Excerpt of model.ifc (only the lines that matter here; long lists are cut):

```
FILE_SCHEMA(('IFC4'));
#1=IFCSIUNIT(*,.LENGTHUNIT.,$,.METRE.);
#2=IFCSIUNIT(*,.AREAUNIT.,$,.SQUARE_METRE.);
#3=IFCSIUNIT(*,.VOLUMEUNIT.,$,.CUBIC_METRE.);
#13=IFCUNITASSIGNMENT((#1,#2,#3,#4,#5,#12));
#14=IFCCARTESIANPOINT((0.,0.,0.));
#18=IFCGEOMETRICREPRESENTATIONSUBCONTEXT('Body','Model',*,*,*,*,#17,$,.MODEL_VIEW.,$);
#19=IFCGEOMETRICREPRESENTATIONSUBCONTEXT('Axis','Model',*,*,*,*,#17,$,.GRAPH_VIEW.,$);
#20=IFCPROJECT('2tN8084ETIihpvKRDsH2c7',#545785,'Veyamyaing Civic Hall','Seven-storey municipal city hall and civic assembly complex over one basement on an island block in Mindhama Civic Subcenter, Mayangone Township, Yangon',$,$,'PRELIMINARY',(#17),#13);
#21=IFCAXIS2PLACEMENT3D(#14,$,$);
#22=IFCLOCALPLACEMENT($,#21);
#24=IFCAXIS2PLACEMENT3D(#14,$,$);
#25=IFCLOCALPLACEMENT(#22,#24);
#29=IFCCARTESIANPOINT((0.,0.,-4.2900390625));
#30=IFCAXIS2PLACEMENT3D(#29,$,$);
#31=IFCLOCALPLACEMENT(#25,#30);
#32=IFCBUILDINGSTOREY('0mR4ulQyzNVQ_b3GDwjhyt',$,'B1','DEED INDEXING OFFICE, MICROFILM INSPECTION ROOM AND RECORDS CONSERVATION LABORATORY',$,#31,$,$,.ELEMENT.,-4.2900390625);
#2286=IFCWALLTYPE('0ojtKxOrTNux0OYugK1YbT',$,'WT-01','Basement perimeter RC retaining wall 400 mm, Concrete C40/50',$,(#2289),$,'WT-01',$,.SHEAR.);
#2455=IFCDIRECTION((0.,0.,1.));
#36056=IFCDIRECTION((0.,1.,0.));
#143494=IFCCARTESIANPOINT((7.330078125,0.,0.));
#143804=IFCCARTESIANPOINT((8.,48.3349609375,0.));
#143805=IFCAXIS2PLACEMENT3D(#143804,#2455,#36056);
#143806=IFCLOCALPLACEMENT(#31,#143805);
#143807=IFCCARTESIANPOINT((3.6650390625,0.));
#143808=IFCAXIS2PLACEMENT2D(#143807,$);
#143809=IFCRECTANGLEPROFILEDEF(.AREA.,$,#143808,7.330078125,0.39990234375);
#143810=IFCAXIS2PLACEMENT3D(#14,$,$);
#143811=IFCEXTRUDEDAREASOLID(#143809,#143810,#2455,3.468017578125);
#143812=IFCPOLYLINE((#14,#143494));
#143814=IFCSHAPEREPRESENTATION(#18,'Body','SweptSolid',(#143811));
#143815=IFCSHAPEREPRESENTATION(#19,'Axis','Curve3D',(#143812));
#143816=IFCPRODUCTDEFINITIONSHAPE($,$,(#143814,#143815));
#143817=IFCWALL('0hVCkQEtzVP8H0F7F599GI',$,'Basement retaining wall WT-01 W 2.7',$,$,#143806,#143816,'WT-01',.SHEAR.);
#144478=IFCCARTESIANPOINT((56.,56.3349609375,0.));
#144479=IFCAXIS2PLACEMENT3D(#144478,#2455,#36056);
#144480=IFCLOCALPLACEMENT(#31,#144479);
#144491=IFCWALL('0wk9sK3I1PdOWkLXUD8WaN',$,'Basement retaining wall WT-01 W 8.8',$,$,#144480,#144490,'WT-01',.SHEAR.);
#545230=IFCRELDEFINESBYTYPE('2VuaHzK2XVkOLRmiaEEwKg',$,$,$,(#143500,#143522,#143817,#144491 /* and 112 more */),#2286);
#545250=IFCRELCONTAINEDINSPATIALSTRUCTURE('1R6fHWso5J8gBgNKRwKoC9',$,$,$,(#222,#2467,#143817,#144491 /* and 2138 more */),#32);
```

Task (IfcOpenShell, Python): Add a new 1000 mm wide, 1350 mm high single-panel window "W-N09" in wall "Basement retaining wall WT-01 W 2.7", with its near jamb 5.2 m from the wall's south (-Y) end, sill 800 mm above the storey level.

```python
import numpy as np
import ifcopenshell
import ifcopenshell.api.feature
import ifcopenshell.api.geometry
import ifcopenshell.api.root
import ifcopenshell.api.spatial
import ifcopenshell.geom
import ifcopenshell.util.element
import ifcopenshell.util.placement
import ifcopenshell.util.representation
import ifcopenshell.util.shape
import ifcopenshell.util.unit

model = ifcopenshell.open("model.ifc")
unit_scale = ifcopenshell.util.unit.calculate_unit_scale(model)
settings = ifcopenshell.geom.settings()


def volume(element):
    """Net volume in cubic metres, openings subtracted."""
    shape = ifcopenshell.geom.create_shape(settings, element)
    return ifcopenshell.util.shape.get_volume(shape.geometry)


wall = model.by_id(143817)
storey = ifcopenshell.util.element.get_container(wall, ifc_class="IfcBuildingStorey")
context = ifcopenshell.util.representation.get_context(model, "Model", "Body", "MODEL_VIEW")
before = volume(wall)

width, height, from_end, sill = 1, 1.35, 5.2, 0.8  # metres

# The wall runs along its own X axis, and the end named is its -X end.
wall_shape = ifcopenshell.geom.create_shape(settings, wall)
x, y, z = ifcopenshell.util.shape.get_vertices(wall_shape.geometry).T
start = x.min() + from_end
face, thickness = float(y.min()), float(y.max() - y.min())
wall_matrix = ifcopenshell.util.placement.get_local_placement(wall.ObjectPlacement)
level = ifcopenshell.util.placement.get_local_placement(storey.ObjectPlacement)[2, 3]


def in_wall(x, y):
    """Placement at x, y metres in the wall's axes, at sill height."""
    matrix = wall_matrix.copy()
    matrix[:, 3] = wall_matrix @ np.array([x / unit_scale, y / unit_scale, 0.0, 1.0])
    matrix[2, 3] = level + sill / unit_scale
    return matrix


# Opening: a box that overshoots both wall faces by 50 mm.
opening = ifcopenshell.api.root.create_entity(model, ifc_class="IfcOpeningElement", predefined_type="OPENING")
box = ifcopenshell.api.geometry.add_wall_representation(
    model, context=context, length=width, height=height, thickness=thickness + 0.1
)
ifcopenshell.api.geometry.assign_representation(model, product=opening, representation=box)
ifcopenshell.api.geometry.edit_object_placement(model, product=opening, matrix=in_wall(start, face - 0.05), is_si=False)
ifcopenshell.api.feature.add_feature(model, feature=opening, element=wall)

window = ifcopenshell.api.root.create_entity(model, ifc_class="IfcWindow", name="W-N09", predefined_type="WINDOW")
window.OverallWidth, window.OverallHeight = width / unit_scale, height / unit_scale
window.PartitioningType = "SINGLE_PANEL"
body = ifcopenshell.api.geometry.add_window_representation(
    model,
    context=context,
    overall_width=window.OverallWidth,
    overall_height=window.OverallHeight,
    partition_type="SINGLE_PANEL",
)
ifcopenshell.api.geometry.assign_representation(model, product=window, representation=body)
ifcopenshell.api.spatial.assign_container(model, products=[window], relating_structure=storey)
ifcopenshell.api.feature.add_filling(model, opening=opening, element=window)

# Centre the window in the wall's thickness.
ifcopenshell.api.geometry.edit_object_placement(model, product=window, matrix=in_wall(start, face), is_si=False)
window_shape = ifcopenshell.geom.create_shape(settings, window)
depth = ifcopenshell.util.shape.get_vertices(window_shape.geometry)[:, 1]
offset = face + thickness / 2 - (depth.min() + depth.max()) / 2
ifcopenshell.api.geometry.edit_object_placement(model, product=window, matrix=in_wall(start, offset), is_si=False)

after = volume(wall)

print(f"wall volume {before:.3f} -> {after:.3f} m3")

model.write("model_v2.ifc")
```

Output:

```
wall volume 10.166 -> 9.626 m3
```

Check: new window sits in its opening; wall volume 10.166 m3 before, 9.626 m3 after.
